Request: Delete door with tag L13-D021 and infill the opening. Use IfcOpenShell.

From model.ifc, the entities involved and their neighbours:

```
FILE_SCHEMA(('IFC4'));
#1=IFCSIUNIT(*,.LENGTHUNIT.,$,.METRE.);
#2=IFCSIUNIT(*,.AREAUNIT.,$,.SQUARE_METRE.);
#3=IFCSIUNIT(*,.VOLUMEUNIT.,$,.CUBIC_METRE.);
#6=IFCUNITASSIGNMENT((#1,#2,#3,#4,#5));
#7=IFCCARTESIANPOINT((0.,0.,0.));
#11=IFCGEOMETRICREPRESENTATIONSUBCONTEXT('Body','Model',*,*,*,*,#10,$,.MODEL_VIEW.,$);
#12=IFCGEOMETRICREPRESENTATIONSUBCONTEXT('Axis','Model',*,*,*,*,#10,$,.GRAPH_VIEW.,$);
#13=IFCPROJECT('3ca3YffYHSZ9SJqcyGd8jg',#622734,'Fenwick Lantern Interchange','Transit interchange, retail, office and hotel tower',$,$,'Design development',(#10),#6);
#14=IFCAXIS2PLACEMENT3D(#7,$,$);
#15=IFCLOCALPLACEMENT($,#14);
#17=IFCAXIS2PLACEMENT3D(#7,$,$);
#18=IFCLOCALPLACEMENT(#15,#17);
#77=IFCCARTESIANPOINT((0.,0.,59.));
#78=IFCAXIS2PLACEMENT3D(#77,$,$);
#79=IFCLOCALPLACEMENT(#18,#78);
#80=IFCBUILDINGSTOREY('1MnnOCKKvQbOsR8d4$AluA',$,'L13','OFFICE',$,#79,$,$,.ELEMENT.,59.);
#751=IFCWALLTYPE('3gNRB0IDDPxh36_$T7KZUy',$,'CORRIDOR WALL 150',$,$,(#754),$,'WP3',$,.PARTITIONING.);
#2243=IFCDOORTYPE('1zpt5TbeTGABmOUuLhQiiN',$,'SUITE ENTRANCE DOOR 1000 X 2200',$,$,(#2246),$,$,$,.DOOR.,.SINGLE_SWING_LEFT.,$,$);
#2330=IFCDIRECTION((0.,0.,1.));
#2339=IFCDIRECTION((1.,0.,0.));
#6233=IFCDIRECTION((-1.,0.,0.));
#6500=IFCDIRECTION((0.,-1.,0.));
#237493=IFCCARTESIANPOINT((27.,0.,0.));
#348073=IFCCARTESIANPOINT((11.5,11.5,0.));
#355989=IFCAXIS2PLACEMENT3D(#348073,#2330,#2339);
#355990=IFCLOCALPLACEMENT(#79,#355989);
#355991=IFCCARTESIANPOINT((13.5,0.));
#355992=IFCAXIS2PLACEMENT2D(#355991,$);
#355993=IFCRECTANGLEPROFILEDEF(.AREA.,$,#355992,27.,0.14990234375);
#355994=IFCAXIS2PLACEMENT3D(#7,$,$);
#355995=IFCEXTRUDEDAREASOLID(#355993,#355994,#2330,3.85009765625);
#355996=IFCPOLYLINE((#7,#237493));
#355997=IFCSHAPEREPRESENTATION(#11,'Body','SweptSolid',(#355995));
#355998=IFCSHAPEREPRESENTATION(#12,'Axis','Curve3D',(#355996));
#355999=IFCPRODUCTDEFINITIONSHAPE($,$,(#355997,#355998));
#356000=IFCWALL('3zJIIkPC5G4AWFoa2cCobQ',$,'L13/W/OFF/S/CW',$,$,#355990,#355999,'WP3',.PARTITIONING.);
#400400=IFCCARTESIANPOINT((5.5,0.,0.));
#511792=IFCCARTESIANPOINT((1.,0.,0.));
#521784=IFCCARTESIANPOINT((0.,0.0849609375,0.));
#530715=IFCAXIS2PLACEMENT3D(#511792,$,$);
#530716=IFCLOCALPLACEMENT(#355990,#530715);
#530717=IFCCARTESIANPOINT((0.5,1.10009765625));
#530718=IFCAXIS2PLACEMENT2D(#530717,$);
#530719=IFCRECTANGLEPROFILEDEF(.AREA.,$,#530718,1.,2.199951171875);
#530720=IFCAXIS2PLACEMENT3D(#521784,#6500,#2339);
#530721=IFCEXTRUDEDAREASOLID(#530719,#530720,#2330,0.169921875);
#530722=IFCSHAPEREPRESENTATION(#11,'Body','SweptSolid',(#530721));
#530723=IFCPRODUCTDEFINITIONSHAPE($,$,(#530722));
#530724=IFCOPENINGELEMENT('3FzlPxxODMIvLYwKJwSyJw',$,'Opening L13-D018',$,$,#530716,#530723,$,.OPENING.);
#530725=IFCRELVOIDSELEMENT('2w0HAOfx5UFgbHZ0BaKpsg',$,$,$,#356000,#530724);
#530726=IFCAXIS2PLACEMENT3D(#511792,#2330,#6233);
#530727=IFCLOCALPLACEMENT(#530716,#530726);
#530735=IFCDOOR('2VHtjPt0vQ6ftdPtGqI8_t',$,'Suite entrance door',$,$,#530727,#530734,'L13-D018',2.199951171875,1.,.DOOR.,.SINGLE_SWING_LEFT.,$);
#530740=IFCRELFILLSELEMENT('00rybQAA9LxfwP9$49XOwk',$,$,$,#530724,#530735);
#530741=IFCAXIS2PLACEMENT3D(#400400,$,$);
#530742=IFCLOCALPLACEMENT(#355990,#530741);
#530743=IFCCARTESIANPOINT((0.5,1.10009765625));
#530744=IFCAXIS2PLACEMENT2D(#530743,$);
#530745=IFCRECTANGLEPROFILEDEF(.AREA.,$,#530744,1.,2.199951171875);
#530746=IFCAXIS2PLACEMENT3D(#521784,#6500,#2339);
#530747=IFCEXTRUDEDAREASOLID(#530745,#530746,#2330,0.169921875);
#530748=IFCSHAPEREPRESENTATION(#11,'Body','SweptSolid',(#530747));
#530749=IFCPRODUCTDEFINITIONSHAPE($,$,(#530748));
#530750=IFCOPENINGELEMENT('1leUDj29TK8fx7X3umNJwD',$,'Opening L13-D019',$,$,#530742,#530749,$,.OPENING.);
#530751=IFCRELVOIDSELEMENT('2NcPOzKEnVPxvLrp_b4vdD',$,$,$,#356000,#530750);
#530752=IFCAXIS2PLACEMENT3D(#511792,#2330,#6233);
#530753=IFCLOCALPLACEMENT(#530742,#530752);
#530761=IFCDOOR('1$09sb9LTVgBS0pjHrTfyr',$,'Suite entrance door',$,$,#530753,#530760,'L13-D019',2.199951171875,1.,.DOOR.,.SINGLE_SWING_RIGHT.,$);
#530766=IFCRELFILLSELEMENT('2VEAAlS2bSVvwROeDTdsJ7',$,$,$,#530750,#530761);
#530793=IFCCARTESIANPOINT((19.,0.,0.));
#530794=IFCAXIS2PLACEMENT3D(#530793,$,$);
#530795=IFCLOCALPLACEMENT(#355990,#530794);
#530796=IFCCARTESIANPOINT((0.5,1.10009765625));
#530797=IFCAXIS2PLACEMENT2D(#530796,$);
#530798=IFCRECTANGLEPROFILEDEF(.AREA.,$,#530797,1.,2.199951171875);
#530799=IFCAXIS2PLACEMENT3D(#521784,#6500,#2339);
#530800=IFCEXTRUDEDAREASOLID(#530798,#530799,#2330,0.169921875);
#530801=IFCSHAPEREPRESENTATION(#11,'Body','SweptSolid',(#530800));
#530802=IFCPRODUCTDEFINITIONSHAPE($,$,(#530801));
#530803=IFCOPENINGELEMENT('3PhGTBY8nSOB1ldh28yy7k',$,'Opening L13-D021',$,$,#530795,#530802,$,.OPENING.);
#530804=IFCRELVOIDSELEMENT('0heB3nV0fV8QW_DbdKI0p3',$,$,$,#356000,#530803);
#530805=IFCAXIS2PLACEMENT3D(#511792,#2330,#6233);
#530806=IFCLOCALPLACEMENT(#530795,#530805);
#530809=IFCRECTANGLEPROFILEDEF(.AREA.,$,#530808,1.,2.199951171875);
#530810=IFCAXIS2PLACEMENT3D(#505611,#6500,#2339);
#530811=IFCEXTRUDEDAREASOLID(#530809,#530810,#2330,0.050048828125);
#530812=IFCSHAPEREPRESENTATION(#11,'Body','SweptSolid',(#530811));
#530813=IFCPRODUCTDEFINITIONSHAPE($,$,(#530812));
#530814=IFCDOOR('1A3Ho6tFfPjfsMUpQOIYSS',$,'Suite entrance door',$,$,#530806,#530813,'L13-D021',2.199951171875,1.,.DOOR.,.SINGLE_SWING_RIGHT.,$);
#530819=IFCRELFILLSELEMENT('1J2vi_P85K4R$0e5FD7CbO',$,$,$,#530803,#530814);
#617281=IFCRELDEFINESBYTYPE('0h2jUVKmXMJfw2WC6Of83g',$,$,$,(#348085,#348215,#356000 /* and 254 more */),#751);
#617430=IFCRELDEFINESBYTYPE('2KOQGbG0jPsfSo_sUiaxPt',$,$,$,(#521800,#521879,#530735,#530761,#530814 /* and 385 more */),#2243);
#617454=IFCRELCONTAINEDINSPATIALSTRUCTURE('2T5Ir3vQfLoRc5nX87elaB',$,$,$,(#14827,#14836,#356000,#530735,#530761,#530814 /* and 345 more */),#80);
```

```python
import ifcopenshell
import ifcopenshell.api.feature
import ifcopenshell.api.root
import ifcopenshell.geom
import ifcopenshell.util.shape

model = ifcopenshell.open("model.ifc")
settings = ifcopenshell.geom.settings()


def volume(element):
    """Net volume in cubic metres, openings subtracted."""
    shape = ifcopenshell.geom.create_shape(settings, element)
    return ifcopenshell.util.shape.get_volume(shape.geometry)


door = model.by_guid("1A3Ho6tFfPjfsMUpQOIYSS")
opening = door.FillsVoids[0].RelatingOpeningElement
wall = opening.VoidsElements[0].RelatingBuildingElement
before = volume(wall)

ifcopenshell.api.root.remove_product(model, product=door)
ifcopenshell.api.feature.remove_feature(model, feature=opening)

after = volume(wall)

print(f"wall volume {before:.3f} -> {after:.3f} m3")

model.write("model-out.ifc")
```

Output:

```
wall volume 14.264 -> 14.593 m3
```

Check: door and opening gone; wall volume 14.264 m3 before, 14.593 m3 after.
